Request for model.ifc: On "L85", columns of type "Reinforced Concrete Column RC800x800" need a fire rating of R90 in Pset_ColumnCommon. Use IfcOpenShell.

First a look at what the model holds.

```python
import ifcopenshell
import ifcopenshell.util.element

model = ifcopenshell.open("model.ifc")
print(model.schema)
storey = next(s for s in model.by_type("IfcBuildingStorey") if s.Name == "L85")
columns = [e for e in ifcopenshell.util.element.get_decomposition(storey) if e.is_a("IfcColumn")]
seen = {}
for e in columns:
    element_type = ifcopenshell.util.element.get_type(e)
    key = (element_type.Name if element_type != e and element_type else None, ifcopenshell.util.element.get_pset(e, "Pset_ColumnCommon", "FireRating"))
    seen[key] = seen.get(key, 0) + 1
for (name, value), count in sorted(seen.items(), key=str):
    print(count, "x", name, "|", value)
```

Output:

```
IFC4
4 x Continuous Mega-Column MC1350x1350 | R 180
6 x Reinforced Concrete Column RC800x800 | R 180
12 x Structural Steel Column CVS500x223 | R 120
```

```python
import ifcopenshell
import ifcopenshell.api.pset
import ifcopenshell.util.element

model = ifcopenshell.open("model.ifc")

storey = next(s for s in model.by_type("IfcBuildingStorey") if s.Name == "L85")
columns = [e for e in ifcopenshell.util.element.get_decomposition(storey) if e.is_a("IfcColumn")]

count = 0
for e in columns:
    element_type = ifcopenshell.util.element.get_type(e)
    if element_type in (None, e) or element_type.Name != "Reinforced Concrete Column RC800x800":
        continue
    found = ifcopenshell.util.element.get_pset(e, "Pset_ColumnCommon", should_inherit=False)
    if found:
        pset = model.by_id(found["id"])
        if len(ifcopenshell.util.element.get_elements_by_pset(pset)) > 1:
            pset = ifcopenshell.api.pset.unshare_pset(model, products=[e], pset=pset)[0]
    else:
        pset = ifcopenshell.api.pset.add_pset(model, product=e, name="Pset_ColumnCommon")
    ifcopenshell.api.pset.edit_pset(model, pset=pset, properties={"FireRating": "R90"})
    count += 1

print(count, "columns updated")

model.write("model_rev.ifc")
```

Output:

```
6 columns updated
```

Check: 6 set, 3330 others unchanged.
